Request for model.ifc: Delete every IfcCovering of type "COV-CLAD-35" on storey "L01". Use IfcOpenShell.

First a look at what the model holds.

```python
import ifcopenshell
import ifcopenshell.util.element

model = ifcopenshell.open("model.ifc")
print(model.schema)
storey = next(s for s in model.by_type("IfcBuildingStorey") if s.Name == "L01")
coverings = [e for e in ifcopenshell.util.element.get_decomposition(storey) if e.is_a("IfcCovering")]
seen = {}
for e in coverings:
    element_type = ifcopenshell.util.element.get_type(e)
    name = element_type.Name if element_type not in (None, e) else None
    seen[name] = seen.get(name, 0) + 1
for name, count in sorted(seen.items(), key=str):
    print(count, "x", name)
```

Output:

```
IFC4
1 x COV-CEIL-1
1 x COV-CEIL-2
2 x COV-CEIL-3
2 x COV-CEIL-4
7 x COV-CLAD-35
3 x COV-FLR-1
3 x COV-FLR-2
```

```python
import ifcopenshell
import ifcopenshell.api.root
import ifcopenshell.util.element

model = ifcopenshell.open("model.ifc")

storey = next(s for s in model.by_type("IfcBuildingStorey") if s.Name == "L01")
coverings = [e for e in ifcopenshell.util.element.get_decomposition(storey) if e.is_a("IfcCovering")]
targets = [e for e in coverings if (t := ifcopenshell.util.element.get_type(e)) not in (None, e) and t.Name == "COV-CLAD-35"]

for e in targets:
    ifcopenshell.api.root.remove_product(model, product=e)
print(len(targets), "removed")

model.write("model_v2.ifc")
```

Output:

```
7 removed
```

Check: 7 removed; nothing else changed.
